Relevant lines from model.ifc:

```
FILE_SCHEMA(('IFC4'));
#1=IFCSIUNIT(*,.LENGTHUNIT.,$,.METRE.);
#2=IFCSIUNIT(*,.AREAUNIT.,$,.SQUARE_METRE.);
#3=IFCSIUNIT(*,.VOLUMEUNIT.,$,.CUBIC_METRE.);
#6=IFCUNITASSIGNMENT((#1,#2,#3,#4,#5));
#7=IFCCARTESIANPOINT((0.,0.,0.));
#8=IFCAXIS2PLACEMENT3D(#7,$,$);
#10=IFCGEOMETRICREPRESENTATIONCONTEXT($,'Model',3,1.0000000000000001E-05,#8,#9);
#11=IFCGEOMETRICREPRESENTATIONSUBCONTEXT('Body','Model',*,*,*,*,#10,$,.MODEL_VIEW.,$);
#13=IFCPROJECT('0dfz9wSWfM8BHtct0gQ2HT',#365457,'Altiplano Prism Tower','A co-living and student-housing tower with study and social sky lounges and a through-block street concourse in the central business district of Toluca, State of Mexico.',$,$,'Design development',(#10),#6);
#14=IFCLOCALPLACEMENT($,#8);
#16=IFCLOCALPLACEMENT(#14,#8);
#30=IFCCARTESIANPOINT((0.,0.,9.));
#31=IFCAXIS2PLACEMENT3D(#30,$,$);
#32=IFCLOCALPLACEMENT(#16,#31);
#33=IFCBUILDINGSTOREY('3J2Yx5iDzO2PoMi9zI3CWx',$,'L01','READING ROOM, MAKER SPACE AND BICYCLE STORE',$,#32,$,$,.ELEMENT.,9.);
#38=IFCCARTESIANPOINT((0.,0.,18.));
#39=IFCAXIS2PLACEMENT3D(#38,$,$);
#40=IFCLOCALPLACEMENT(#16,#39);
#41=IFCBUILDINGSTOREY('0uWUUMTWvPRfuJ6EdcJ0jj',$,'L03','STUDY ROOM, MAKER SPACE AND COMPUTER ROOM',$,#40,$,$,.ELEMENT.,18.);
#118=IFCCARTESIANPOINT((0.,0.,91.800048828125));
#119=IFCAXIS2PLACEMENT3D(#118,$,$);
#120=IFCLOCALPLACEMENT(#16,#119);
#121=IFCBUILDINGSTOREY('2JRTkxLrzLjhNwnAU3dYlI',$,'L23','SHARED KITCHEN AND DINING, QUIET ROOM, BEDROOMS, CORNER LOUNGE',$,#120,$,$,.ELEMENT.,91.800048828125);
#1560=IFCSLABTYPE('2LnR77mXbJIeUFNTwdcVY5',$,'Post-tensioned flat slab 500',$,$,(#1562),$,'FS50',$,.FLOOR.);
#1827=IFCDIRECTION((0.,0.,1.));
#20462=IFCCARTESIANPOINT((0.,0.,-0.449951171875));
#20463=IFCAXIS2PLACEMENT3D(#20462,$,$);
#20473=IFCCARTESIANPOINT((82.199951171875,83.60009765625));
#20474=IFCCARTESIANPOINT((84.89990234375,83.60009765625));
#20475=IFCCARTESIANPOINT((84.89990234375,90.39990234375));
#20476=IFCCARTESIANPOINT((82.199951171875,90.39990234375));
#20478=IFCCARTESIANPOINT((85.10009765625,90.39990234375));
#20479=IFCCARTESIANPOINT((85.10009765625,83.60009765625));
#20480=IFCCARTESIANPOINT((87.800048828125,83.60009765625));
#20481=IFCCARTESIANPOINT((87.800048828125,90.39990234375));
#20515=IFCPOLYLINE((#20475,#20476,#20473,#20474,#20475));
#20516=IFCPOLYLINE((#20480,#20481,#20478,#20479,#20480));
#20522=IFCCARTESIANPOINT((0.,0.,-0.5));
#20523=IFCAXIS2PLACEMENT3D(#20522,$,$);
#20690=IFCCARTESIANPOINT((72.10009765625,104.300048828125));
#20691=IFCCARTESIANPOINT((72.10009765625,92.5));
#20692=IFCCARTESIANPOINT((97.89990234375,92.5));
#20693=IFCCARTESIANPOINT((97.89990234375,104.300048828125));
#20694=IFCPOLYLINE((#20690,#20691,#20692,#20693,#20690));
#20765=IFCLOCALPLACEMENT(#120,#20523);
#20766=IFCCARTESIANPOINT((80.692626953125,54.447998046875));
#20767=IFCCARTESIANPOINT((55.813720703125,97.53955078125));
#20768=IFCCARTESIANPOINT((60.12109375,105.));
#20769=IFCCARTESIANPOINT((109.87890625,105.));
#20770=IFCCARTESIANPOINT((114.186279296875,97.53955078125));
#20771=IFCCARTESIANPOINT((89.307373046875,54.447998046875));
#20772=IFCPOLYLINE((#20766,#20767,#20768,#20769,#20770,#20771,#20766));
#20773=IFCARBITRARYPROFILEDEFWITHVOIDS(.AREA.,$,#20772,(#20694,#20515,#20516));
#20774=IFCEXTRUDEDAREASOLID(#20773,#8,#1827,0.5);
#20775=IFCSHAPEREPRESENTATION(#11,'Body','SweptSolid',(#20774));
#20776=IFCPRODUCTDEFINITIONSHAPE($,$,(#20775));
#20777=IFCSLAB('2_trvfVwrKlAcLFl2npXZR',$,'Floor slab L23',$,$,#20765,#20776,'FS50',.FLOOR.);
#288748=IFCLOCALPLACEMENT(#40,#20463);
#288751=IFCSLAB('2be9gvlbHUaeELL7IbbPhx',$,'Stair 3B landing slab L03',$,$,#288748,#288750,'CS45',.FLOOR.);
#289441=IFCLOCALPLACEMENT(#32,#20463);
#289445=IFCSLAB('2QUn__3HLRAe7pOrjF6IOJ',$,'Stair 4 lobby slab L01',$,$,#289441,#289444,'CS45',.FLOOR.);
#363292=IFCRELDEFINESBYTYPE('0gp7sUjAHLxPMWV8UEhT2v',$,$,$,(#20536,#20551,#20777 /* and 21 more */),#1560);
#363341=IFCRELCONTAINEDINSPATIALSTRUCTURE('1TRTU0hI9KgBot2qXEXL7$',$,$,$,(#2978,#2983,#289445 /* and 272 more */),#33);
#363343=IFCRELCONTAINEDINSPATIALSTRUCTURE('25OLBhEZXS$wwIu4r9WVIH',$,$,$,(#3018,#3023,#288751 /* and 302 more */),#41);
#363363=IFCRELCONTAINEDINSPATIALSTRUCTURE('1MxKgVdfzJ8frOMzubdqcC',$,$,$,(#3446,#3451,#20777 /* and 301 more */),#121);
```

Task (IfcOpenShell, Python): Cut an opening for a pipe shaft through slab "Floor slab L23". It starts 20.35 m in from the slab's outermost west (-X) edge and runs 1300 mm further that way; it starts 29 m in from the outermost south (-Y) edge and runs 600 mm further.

```python
import numpy as np
import ifcopenshell
import ifcopenshell.api.feature
import ifcopenshell.api.geometry
import ifcopenshell.api.root
import ifcopenshell.geom
import ifcopenshell.util.placement
import ifcopenshell.util.representation
import ifcopenshell.util.shape
import ifcopenshell.util.unit

model = ifcopenshell.open("model.ifc")
unit_scale = ifcopenshell.util.unit.calculate_unit_scale(model)
settings = ifcopenshell.geom.settings()


def volume(element):
    """Net volume in cubic metres, openings subtracted."""
    shape = ifcopenshell.geom.create_shape(settings, element)
    return ifcopenshell.util.shape.get_volume(shape.geometry)


slab = model.by_guid("2_trvfVwrKlAcLFl2npXZR")
before = volume(slab)

# Extent in the slab's own axes, in metres. The edges named are its -X and -Y sides.
slab_shape = ifcopenshell.geom.create_shape(settings, slab)
vertices = ifcopenshell.util.shape.get_vertices(slab_shape.geometry)
x_min, y_min, bottom = vertices.min(axis=0)
top = vertices[:, 2].max()

opening = ifcopenshell.api.root.create_entity(model, ifc_class="IfcOpeningElement", name="Pipe shaft opening", predefined_type="OPENING")
context = ifcopenshell.util.representation.get_context(model, "Model", "Body", "MODEL_VIEW")
width, depth = 1.3, 0.6
outline = [(0.0, 0.0), (width, 0.0), (width, depth), (0.0, depth), (0.0, 0.0)]
# Overshoot both faces by 50 mm so the cut is clean.
shape = ifcopenshell.api.geometry.add_slab_representation(
    model, context=context, depth=top - bottom + 0.1, polyline=outline
)
ifcopenshell.api.geometry.assign_representation(model, product=opening, representation=shape)

matrix = ifcopenshell.util.placement.get_local_placement(slab.ObjectPlacement)
matrix[:, 3] = matrix @ np.append(np.array([x_min + 20.35, y_min + 29, bottom - 0.05]) / unit_scale, 1.0)
ifcopenshell.api.geometry.edit_object_placement(model, product=opening, matrix=matrix, is_si=False)
ifcopenshell.api.feature.add_feature(model, feature=opening, element=slab)

after = volume(slab)

print(f"slab volume {before:.3f} -> {after:.3f} m3")

model.write("model-out.ifc")
```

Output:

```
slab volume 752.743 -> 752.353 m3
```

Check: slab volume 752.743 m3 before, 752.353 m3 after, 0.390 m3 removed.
